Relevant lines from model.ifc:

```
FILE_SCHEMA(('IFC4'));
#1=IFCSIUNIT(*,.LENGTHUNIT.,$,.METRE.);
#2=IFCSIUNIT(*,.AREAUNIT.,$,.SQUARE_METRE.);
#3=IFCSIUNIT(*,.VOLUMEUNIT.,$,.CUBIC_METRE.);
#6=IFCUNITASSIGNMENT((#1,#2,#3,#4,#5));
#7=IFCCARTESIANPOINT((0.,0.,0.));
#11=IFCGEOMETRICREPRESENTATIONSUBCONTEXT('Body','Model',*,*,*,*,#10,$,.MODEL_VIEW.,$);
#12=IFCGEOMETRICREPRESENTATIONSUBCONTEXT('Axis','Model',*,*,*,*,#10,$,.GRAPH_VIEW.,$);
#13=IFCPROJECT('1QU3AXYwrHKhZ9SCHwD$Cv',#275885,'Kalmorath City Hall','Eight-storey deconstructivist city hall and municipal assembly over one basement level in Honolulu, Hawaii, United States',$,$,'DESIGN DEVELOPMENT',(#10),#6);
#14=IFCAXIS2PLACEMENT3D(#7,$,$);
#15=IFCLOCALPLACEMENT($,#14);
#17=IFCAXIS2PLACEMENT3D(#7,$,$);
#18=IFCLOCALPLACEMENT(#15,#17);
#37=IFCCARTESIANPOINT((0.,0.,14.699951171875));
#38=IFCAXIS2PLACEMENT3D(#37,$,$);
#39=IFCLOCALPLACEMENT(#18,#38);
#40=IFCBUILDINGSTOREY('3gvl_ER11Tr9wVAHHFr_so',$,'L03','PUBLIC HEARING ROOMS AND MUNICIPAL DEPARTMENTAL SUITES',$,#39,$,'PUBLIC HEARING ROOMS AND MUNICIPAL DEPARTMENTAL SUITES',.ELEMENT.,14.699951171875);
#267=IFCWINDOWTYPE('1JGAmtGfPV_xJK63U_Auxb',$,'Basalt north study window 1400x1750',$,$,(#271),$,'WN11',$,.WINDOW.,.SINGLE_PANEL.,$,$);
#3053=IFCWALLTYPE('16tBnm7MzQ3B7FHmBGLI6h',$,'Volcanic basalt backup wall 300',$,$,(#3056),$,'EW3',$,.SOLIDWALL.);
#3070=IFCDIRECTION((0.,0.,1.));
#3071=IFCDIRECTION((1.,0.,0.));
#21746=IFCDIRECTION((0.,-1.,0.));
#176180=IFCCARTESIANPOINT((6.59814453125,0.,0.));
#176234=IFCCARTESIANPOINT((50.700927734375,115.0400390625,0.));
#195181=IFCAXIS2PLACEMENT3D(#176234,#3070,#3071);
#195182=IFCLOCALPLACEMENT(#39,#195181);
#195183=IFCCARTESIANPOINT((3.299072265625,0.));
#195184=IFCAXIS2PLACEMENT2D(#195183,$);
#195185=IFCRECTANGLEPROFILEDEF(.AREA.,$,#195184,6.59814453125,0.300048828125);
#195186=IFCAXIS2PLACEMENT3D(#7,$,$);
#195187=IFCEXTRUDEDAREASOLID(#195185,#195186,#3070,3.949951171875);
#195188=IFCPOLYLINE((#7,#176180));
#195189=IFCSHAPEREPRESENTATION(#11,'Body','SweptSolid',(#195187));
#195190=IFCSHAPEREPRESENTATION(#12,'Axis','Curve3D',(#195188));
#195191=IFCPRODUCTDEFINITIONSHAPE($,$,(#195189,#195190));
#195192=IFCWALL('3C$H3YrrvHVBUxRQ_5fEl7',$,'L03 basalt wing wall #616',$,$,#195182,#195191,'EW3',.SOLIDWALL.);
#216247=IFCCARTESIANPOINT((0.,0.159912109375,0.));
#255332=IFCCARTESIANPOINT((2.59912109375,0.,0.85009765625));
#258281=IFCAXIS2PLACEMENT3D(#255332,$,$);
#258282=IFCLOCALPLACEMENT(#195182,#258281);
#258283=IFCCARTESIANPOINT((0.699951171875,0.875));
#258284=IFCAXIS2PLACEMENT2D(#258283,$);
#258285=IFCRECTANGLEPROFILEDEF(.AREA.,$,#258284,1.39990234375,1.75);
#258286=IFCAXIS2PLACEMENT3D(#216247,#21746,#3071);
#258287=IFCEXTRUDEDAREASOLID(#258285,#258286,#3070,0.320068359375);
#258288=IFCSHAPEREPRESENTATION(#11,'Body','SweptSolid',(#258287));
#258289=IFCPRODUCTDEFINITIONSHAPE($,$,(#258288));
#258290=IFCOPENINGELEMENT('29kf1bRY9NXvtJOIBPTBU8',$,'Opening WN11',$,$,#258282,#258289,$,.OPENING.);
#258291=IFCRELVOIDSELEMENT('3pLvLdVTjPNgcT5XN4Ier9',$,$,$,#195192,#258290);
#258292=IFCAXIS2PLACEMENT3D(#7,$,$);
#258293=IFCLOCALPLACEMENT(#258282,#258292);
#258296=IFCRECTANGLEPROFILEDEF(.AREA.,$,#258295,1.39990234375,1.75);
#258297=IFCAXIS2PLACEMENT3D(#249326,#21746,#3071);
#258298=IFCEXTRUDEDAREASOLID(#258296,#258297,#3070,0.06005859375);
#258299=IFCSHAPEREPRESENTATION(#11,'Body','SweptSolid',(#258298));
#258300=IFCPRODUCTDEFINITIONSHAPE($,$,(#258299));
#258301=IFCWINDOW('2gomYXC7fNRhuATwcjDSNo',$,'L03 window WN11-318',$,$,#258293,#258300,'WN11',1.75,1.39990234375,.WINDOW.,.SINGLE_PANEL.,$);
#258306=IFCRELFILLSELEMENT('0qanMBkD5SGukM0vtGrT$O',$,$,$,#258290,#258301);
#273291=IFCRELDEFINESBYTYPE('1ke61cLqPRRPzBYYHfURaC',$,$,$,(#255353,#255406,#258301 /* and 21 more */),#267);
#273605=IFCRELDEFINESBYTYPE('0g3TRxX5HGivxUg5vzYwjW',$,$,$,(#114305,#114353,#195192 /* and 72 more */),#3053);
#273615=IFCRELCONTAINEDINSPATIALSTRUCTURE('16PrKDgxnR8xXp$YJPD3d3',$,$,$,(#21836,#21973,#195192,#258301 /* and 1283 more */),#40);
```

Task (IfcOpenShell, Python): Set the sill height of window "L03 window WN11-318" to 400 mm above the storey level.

```python
import numpy as np
import ifcopenshell
import ifcopenshell.api.geometry
import ifcopenshell.geom
import ifcopenshell.util.element
import ifcopenshell.util.placement
import ifcopenshell.util.shape
import ifcopenshell.util.unit

model = ifcopenshell.open("model.ifc")
unit_scale = ifcopenshell.util.unit.calculate_unit_scale(model)

window = model.by_guid("2gomYXC7fNRhuATwcjDSNo")
opening = window.FillsVoids[0].RelatingOpeningElement
storey = ifcopenshell.util.element.get_container(window, ifc_class="IfcBuildingStorey")
level = ifcopenshell.util.placement.get_local_placement(storey.ObjectPlacement)[2, 3]

# The opening's origin need not be at the sill, so measure its lowest point.
shape = ifcopenshell.geom.create_shape(ifcopenshell.geom.settings(), opening)
bottom = ifcopenshell.util.shape.get_shape_bottom_elevation(shape, shape.geometry) / unit_scale
dz = level + 0.4 - bottom

shift = np.array([0.0, 0.0, dz])
# The window is placed relative to its opening, so it follows when the opening moves.
matrix = ifcopenshell.util.placement.get_local_placement(opening.ObjectPlacement)
matrix[:3, 3] += shift
ifcopenshell.api.geometry.edit_object_placement(
    model, product=opening, matrix=matrix, is_si=False, should_transform_children=True
)

print(f"moved by {dz * unit_scale:+.3f} m")

model.write("model-out.ifc")
```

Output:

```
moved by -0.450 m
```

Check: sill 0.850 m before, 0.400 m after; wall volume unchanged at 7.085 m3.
